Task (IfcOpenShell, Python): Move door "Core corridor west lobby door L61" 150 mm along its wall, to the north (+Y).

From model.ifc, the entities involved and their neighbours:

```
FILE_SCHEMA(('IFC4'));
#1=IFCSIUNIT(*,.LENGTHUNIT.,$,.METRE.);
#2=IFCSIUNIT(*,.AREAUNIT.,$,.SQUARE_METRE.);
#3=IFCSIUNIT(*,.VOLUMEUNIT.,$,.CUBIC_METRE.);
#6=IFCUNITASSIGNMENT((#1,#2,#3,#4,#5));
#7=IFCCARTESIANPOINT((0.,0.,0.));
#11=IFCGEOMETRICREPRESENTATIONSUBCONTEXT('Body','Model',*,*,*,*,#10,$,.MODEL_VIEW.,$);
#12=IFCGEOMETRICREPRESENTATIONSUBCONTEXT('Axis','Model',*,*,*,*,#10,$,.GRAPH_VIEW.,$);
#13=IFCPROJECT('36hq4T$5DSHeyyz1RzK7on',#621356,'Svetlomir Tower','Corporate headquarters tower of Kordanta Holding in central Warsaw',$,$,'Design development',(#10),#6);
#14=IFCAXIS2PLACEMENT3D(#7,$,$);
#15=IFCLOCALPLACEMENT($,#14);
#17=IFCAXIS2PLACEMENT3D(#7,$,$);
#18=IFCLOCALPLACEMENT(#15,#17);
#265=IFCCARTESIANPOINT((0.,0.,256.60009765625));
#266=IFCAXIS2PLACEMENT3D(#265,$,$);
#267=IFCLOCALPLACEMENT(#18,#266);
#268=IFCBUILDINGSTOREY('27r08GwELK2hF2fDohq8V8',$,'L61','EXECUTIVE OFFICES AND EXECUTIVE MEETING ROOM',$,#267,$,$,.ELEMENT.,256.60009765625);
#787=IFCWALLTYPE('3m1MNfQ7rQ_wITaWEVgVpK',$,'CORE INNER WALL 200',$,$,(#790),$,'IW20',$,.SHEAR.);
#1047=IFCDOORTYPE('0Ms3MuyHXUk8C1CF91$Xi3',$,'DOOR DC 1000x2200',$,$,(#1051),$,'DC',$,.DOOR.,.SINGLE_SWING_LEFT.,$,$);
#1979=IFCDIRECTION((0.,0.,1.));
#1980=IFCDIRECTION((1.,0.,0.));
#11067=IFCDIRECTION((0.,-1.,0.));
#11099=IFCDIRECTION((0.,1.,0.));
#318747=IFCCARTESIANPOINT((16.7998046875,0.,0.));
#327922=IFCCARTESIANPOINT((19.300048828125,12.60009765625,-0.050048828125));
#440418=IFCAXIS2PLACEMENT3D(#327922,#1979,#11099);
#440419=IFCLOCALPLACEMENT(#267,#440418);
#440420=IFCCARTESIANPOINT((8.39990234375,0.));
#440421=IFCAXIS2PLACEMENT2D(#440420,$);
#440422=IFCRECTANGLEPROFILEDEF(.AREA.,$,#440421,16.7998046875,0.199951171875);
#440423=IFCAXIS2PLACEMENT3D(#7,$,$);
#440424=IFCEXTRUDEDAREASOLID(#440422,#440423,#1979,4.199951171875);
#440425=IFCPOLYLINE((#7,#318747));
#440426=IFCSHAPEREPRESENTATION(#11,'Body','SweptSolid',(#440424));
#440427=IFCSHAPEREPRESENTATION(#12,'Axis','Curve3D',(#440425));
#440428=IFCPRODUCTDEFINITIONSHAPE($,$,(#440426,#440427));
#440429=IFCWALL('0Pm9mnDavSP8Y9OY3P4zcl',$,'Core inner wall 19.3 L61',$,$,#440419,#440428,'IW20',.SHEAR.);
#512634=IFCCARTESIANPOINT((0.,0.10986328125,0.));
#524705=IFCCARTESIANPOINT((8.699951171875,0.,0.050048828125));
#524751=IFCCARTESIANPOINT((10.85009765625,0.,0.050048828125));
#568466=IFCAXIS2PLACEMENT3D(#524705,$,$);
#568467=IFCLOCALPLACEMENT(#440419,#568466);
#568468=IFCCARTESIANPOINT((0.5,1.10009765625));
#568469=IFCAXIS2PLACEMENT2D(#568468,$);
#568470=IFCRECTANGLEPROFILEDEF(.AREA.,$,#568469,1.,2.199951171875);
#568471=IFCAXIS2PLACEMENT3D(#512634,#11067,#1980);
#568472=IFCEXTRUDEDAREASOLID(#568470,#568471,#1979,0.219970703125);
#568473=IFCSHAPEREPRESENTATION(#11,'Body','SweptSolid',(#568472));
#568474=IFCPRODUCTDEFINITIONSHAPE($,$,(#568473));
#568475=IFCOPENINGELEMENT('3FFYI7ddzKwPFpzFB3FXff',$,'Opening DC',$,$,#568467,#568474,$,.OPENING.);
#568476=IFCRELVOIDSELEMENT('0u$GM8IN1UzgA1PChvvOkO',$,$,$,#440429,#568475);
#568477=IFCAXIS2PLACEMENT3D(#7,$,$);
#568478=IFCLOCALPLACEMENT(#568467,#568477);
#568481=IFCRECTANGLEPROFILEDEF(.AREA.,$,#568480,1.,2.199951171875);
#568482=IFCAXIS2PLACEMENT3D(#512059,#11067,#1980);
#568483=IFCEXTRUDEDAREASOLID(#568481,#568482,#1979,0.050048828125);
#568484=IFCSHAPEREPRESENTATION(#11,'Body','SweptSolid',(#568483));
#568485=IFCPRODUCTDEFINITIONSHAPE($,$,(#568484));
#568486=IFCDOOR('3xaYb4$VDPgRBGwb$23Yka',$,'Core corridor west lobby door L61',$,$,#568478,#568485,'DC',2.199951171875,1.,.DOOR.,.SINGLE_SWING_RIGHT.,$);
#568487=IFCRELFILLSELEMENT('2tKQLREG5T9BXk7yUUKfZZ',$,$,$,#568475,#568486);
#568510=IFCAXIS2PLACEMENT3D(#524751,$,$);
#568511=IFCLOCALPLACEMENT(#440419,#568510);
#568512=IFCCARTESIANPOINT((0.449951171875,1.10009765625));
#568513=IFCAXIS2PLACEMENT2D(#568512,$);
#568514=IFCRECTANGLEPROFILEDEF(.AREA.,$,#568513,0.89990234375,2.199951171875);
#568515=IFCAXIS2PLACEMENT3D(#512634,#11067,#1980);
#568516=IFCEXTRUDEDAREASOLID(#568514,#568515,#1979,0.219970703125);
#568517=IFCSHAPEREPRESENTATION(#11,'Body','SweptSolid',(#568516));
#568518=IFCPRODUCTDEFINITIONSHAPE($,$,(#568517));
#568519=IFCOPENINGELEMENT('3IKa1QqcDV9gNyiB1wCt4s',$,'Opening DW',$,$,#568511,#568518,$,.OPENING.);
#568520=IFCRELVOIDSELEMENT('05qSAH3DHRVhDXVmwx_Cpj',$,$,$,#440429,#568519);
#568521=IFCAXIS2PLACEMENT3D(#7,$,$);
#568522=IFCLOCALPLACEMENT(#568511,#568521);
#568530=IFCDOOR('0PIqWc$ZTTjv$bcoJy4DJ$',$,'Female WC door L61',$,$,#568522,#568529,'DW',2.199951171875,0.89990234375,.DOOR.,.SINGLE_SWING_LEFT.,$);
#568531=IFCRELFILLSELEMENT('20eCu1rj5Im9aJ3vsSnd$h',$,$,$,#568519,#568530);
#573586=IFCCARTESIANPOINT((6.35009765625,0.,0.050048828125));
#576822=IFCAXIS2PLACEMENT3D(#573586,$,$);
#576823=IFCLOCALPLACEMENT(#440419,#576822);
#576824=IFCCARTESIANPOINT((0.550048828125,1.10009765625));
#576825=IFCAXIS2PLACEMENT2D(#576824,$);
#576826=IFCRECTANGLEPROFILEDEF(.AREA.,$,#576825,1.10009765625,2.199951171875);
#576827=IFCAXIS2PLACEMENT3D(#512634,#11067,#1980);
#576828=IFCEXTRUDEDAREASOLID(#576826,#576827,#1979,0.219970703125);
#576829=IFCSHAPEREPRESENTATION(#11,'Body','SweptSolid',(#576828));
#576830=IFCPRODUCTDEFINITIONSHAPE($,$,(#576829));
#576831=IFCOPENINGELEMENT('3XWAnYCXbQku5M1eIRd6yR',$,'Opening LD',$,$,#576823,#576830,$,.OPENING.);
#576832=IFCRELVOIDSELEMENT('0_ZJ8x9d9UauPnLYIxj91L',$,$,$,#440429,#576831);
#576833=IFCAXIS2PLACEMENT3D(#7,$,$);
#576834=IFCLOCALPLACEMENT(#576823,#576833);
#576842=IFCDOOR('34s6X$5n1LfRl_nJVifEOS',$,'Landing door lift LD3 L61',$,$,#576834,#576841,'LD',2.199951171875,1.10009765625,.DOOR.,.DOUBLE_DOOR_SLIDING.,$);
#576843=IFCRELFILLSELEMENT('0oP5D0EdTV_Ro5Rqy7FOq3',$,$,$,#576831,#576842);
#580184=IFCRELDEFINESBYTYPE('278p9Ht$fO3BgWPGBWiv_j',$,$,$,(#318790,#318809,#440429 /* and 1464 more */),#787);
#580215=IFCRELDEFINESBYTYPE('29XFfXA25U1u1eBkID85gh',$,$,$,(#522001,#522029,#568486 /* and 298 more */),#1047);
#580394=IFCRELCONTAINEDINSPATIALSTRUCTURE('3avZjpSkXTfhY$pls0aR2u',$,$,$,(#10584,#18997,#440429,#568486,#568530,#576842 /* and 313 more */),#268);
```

```python
import ifcopenshell
import ifcopenshell.api.geometry
import ifcopenshell.util.placement

model = ifcopenshell.open("model.ifc")

door = model.by_guid("3xaYb4$VDPgRBGwb$23Yka")
opening = door.FillsVoids[0].RelatingOpeningElement
wall = opening.VoidsElements[0].RelatingBuildingElement

wall_matrix = ifcopenshell.util.placement.get_local_placement(wall.ObjectPlacement)
shift = wall_matrix[:3, 0] * 0.15
before = ifcopenshell.util.placement.get_local_placement(door.ObjectPlacement)[:3, 3].copy()

# The door is placed relative to its opening, so it follows when the opening moves.
matrix = ifcopenshell.util.placement.get_local_placement(opening.ObjectPlacement)
matrix[:3, 3] += shift
ifcopenshell.api.geometry.edit_object_placement(
    model, product=opening, matrix=matrix, is_si=False, should_transform_children=True
)

after = ifcopenshell.util.placement.get_local_placement(door.ObjectPlacement)[:3, 3]
print("door moved by", (after - before).round(3) + 0.0)

model.write("model_rev.ifc")
```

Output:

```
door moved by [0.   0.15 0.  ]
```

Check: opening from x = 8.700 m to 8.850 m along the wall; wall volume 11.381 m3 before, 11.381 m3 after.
